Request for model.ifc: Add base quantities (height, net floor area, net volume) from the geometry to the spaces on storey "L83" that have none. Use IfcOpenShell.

First a look at what the model holds.

```python
import ifcopenshell
import ifcopenshell.util.element
import ifcopenshell.util.unit

model = ifcopenshell.open("model.ifc")
print(model.schema)
for unit_type in ("LENGTHUNIT", "AREAUNIT", "VOLUMEUNIT"):
    print(unit_type, ifcopenshell.util.unit.calculate_unit_scale(model, unit_type))
storey = next(s for s in model.by_type("IfcBuildingStorey") if s.Name == "L83")
spaces = [e for e in ifcopenshell.util.element.get_decomposition(storey) if e.is_a("IfcSpace")]
for e in sorted(spaces, key=lambda e: e.id()):
    print(e.id(), e.is_a(), e.Name, list(ifcopenshell.util.element.get_psets(e, qtos_only=True)), sep=" | ")
```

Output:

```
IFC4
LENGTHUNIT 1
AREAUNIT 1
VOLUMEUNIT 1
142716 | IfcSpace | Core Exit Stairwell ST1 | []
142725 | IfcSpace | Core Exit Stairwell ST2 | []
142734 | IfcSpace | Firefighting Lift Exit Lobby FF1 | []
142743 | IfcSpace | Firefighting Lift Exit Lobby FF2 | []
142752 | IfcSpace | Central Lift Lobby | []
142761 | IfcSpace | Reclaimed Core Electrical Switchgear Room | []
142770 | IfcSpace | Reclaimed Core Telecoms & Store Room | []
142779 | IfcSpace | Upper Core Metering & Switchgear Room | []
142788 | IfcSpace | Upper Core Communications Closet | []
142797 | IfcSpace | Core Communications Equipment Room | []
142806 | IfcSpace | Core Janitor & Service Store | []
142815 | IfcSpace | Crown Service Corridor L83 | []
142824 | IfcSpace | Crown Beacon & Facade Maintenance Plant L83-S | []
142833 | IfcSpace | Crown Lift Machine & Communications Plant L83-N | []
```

```python
import ifcopenshell
import ifcopenshell.api.pset
import ifcopenshell.geom
import ifcopenshell.util.element
import ifcopenshell.util.shape
import ifcopenshell.util.unit

model = ifcopenshell.open("model.ifc")
unit_scale = ifcopenshell.util.unit.calculate_unit_scale(model)
area_scale = ifcopenshell.util.unit.calculate_unit_scale(model, "AREAUNIT")
volume_scale = ifcopenshell.util.unit.calculate_unit_scale(model, "VOLUMEUNIT")
settings = ifcopenshell.geom.settings()

storey = next(s for s in model.by_type("IfcBuildingStorey") if s.Name == "L83")
spaces = [e for e in ifcopenshell.util.element.get_decomposition(storey) if e.is_a("IfcSpace")]

for e in sorted(spaces, key=lambda e: e.id()):
    if ifcopenshell.util.element.get_psets(e, qtos_only=True, should_inherit=False):
        continue
    # Geometry comes back in metres, in the element's own axes.
    shape = ifcopenshell.geom.create_shape(settings, e)
    values = {
        "Height": ifcopenshell.util.shape.get_z(shape.geometry) / unit_scale,
        "NetFloorArea": ifcopenshell.util.shape.get_footprint_area(shape.geometry) / area_scale,
        "NetVolume": ifcopenshell.util.shape.get_volume(shape.geometry) / volume_scale,
    }
    qto = ifcopenshell.api.pset.add_qto(model, product=e, name="Qto_SpaceBaseQuantities")
    ifcopenshell.api.pset.edit_qto(model, qto=qto, properties=values)
    print(e.id(), {k: round(v, 3) for k, v in values.items()})

model.write("model-out.ifc")
```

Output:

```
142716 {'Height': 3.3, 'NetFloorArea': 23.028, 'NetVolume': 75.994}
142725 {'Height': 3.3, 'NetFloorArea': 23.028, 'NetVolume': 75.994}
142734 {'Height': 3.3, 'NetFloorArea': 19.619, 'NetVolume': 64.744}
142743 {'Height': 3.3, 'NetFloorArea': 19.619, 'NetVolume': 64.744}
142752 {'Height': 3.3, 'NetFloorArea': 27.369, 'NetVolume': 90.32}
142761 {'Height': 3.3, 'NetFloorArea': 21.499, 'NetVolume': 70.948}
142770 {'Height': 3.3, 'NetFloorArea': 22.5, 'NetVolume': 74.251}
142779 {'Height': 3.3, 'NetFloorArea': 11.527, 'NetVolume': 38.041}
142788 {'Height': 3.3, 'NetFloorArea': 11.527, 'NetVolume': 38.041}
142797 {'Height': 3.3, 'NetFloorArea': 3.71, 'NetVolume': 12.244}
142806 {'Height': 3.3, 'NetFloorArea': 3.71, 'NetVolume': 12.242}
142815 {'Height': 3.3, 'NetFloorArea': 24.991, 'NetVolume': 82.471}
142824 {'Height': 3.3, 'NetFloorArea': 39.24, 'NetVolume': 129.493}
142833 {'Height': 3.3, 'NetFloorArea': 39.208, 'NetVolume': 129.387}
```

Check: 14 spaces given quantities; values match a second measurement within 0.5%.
